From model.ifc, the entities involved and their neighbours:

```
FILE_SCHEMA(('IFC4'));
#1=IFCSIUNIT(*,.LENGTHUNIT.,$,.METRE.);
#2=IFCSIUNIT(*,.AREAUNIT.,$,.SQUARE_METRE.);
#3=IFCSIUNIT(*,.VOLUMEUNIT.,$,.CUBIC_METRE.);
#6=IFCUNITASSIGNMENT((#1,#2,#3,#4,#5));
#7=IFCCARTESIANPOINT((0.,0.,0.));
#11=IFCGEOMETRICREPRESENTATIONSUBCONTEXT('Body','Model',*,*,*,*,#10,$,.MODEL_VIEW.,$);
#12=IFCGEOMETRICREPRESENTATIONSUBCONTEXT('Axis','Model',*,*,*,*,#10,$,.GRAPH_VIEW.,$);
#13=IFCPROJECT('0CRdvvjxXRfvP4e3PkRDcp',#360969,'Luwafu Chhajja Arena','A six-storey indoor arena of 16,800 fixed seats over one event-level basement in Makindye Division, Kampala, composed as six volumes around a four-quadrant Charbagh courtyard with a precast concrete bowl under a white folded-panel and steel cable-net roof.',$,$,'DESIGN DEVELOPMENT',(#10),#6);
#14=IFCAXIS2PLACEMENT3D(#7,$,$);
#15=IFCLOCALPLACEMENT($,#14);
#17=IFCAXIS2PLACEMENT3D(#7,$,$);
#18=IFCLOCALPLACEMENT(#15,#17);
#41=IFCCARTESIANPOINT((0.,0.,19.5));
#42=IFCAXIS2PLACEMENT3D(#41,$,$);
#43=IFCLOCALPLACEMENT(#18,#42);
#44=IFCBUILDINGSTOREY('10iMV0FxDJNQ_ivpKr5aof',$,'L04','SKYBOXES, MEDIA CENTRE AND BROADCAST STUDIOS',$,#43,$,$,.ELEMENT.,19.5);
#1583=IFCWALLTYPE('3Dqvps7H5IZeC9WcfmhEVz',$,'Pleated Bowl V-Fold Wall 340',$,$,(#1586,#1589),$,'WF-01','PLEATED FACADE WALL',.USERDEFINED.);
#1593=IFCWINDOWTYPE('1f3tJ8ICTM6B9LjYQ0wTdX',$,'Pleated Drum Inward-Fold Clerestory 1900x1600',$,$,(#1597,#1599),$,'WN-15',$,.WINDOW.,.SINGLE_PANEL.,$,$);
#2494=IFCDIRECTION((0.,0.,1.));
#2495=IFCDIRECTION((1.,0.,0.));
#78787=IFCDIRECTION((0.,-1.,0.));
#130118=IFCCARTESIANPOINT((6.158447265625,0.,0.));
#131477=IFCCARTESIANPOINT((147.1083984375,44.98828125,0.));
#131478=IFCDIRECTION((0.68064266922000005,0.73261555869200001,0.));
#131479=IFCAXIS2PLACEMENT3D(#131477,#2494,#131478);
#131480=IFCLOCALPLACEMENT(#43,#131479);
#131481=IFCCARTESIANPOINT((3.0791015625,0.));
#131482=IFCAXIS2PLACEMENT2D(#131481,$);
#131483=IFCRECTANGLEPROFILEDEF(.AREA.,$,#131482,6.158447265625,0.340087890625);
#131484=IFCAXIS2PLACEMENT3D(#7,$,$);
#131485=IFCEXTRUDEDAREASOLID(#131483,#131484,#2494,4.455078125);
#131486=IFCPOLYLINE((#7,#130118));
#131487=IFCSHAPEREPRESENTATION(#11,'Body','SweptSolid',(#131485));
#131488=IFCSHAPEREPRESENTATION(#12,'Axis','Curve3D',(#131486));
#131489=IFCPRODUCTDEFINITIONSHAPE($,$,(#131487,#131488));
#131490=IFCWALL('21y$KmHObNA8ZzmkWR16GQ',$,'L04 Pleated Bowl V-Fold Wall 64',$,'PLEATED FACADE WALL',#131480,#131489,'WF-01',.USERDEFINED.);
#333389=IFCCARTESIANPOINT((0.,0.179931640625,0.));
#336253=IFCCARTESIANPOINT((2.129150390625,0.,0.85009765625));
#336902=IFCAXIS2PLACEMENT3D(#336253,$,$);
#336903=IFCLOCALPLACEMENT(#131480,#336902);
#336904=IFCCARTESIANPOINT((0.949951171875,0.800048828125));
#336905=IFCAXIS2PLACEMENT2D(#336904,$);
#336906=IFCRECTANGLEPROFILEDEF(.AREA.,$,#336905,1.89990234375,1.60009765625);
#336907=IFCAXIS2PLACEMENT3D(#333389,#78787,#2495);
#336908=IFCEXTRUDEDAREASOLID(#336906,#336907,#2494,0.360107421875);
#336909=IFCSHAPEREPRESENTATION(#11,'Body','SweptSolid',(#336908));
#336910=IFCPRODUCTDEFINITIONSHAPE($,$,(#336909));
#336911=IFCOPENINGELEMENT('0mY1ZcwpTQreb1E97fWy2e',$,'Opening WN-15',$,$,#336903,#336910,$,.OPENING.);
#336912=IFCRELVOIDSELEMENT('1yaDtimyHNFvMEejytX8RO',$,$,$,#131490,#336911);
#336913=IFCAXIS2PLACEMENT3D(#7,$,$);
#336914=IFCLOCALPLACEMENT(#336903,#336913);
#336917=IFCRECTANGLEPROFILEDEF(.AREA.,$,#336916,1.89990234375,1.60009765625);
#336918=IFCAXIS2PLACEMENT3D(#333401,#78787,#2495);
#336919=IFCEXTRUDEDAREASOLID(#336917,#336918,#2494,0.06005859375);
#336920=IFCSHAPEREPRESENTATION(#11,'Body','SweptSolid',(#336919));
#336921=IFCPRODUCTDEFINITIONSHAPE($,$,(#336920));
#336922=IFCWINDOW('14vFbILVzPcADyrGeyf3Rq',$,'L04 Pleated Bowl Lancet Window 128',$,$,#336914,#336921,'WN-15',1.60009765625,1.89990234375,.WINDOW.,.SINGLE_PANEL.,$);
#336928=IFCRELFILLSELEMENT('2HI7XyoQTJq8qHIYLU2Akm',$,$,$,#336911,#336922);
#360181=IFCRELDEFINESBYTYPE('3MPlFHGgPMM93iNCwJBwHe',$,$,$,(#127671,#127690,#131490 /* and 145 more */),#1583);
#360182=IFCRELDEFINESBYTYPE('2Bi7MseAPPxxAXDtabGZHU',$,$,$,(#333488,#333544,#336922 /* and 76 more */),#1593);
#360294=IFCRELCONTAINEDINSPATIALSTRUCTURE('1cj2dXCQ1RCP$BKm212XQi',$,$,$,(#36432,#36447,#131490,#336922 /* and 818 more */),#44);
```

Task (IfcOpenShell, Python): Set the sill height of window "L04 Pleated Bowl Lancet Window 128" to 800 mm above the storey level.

```python
import numpy as np
import ifcopenshell
import ifcopenshell.api.geometry
import ifcopenshell.geom
import ifcopenshell.util.element
import ifcopenshell.util.placement
import ifcopenshell.util.shape
import ifcopenshell.util.unit

model = ifcopenshell.open("model.ifc")
unit_scale = ifcopenshell.util.unit.calculate_unit_scale(model)

window = model.by_id(336922)
opening = window.FillsVoids[0].RelatingOpeningElement
storey = ifcopenshell.util.element.get_container(window, ifc_class="IfcBuildingStorey")
level = ifcopenshell.util.placement.get_local_placement(storey.ObjectPlacement)[2, 3]

# The opening's origin need not be at the sill, so measure its lowest point.
shape = ifcopenshell.geom.create_shape(ifcopenshell.geom.settings(), opening)
bottom = ifcopenshell.util.shape.get_shape_bottom_elevation(shape, shape.geometry) / unit_scale
dz = level + 0.8 - bottom

shift = np.array([0.0, 0.0, dz])
# The window is placed relative to its opening, so it follows when the opening moves.
matrix = ifcopenshell.util.placement.get_local_placement(opening.ObjectPlacement)
matrix[:3, 3] += shift
ifcopenshell.api.geometry.edit_object_placement(
    model, product=opening, matrix=matrix, is_si=False, should_transform_children=True
)

print(f"moved by {dz * unit_scale:+.3f} m")

model.write("model_edited.ifc")
```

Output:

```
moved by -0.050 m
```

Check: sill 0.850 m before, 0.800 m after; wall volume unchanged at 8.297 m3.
